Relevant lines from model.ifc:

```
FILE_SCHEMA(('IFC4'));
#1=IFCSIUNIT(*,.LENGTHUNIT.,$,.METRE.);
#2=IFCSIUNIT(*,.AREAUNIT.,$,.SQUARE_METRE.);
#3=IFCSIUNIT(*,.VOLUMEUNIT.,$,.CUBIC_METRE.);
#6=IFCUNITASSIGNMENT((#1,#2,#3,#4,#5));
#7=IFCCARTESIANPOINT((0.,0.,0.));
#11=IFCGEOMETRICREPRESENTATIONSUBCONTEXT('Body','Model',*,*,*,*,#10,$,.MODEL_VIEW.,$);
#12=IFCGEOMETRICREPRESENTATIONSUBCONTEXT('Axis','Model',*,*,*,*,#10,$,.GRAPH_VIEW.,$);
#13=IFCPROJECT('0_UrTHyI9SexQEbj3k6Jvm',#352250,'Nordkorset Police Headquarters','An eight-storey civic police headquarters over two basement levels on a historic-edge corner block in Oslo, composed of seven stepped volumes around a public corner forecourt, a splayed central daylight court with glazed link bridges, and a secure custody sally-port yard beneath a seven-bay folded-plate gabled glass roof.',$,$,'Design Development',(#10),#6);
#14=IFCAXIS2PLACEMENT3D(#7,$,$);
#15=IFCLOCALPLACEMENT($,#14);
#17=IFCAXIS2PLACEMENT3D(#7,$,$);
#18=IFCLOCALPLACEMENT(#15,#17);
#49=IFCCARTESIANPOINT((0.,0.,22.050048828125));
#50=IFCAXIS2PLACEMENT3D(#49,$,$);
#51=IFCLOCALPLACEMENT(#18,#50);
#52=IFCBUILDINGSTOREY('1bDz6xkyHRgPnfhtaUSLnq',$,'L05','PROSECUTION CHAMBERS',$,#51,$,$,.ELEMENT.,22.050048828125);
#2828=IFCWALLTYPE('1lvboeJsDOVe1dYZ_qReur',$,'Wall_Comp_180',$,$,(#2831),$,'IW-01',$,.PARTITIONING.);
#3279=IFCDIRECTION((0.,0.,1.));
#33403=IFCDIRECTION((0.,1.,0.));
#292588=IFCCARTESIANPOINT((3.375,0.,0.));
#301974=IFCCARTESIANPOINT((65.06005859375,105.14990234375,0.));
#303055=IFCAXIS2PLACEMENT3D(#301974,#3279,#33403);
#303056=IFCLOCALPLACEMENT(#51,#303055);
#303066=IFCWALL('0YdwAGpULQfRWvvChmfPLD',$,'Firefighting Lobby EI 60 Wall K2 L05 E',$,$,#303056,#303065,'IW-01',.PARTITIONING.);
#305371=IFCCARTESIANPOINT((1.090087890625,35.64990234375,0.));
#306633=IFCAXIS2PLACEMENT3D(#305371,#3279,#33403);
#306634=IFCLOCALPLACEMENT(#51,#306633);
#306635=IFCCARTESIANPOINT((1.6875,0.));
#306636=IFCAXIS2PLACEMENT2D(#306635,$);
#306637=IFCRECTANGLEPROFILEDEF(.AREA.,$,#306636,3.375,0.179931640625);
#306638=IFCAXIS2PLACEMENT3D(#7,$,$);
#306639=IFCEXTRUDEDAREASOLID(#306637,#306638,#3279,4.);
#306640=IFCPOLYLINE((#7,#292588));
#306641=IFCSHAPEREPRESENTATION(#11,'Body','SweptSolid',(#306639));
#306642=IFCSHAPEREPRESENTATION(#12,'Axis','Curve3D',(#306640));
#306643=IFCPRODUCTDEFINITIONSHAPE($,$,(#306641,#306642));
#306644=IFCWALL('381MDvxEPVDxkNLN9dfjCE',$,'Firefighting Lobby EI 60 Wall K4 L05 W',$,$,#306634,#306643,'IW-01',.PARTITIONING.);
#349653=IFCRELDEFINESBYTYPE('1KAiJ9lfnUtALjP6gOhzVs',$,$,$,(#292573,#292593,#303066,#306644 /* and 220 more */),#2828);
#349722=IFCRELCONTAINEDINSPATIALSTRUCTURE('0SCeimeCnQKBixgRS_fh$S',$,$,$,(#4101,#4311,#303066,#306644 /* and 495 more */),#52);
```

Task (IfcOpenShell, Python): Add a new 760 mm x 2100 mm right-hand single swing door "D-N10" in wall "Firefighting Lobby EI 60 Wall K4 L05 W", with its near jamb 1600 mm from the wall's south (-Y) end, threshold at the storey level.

```python
import numpy as np
import ifcopenshell
import ifcopenshell.api.feature
import ifcopenshell.api.geometry
import ifcopenshell.api.root
import ifcopenshell.api.spatial
import ifcopenshell.geom
import ifcopenshell.util.element
import ifcopenshell.util.placement
import ifcopenshell.util.representation
import ifcopenshell.util.shape
import ifcopenshell.util.unit

model = ifcopenshell.open("model.ifc")
unit_scale = ifcopenshell.util.unit.calculate_unit_scale(model)
settings = ifcopenshell.geom.settings()


def volume(element):
    """Net volume in cubic metres, openings subtracted."""
    shape = ifcopenshell.geom.create_shape(settings, element)
    return ifcopenshell.util.shape.get_volume(shape.geometry)


wall = model.by_id(306644)
storey = ifcopenshell.util.element.get_container(wall, ifc_class="IfcBuildingStorey")
context = ifcopenshell.util.representation.get_context(model, "Model", "Body", "MODEL_VIEW")
before = volume(wall)

width, height, from_end, sill = 0.76, 2.1, 1.6, 0.0  # metres

# The wall runs along its own X axis, and the end named is its -X end.
wall_shape = ifcopenshell.geom.create_shape(settings, wall)
x, y, z = ifcopenshell.util.shape.get_vertices(wall_shape.geometry).T
start = x.min() + from_end
face, thickness = float(y.min()), float(y.max() - y.min())
wall_matrix = ifcopenshell.util.placement.get_local_placement(wall.ObjectPlacement)
level = ifcopenshell.util.placement.get_local_placement(storey.ObjectPlacement)[2, 3]


def in_wall(x, y):
    """Placement at x, y metres in the wall's axes, at sill height."""
    matrix = wall_matrix.copy()
    matrix[:, 3] = wall_matrix @ np.array([x / unit_scale, y / unit_scale, 0.0, 1.0])
    matrix[2, 3] = level + sill / unit_scale
    return matrix


# Opening: a box that overshoots both wall faces by 50 mm.
opening = ifcopenshell.api.root.create_entity(model, ifc_class="IfcOpeningElement", predefined_type="OPENING")
box = ifcopenshell.api.geometry.add_wall_representation(
    model, context=context, length=width, height=height, thickness=thickness + 0.1
)
ifcopenshell.api.geometry.assign_representation(model, product=opening, representation=box)
ifcopenshell.api.geometry.edit_object_placement(model, product=opening, matrix=in_wall(start, face - 0.05), is_si=False)
ifcopenshell.api.feature.add_feature(model, feature=opening, element=wall)

door = ifcopenshell.api.root.create_entity(model, ifc_class="IfcDoor", name="D-N10", predefined_type="DOOR")
door.OverallWidth, door.OverallHeight = width / unit_scale, height / unit_scale
door.OperationType = "SINGLE_SWING_RIGHT"
body = ifcopenshell.api.geometry.add_door_representation(
    model,
    context=context,
    overall_width=door.OverallWidth,
    overall_height=door.OverallHeight,
    operation_type="SINGLE_SWING_RIGHT",
    lining_properties={"LiningDepth": thickness / unit_scale, "ThresholdDepth": thickness / unit_scale},
)
ifcopenshell.api.geometry.assign_representation(model, product=door, representation=body)
ifcopenshell.api.spatial.assign_container(model, products=[door], relating_structure=storey)
ifcopenshell.api.feature.add_filling(model, opening=opening, element=door)

# The lining spans the wall, so the door starts at the wall face.
ifcopenshell.api.geometry.edit_object_placement(model, product=door, matrix=in_wall(start, face), is_si=False)

after = volume(wall)

print(f"wall volume {before:.3f} -> {after:.3f} m3")

model.write("model-out.ifc")
```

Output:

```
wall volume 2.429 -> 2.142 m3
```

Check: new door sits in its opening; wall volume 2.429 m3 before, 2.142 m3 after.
